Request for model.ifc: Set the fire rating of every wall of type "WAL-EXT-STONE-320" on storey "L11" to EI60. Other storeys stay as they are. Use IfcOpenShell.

First a look at what the model holds.

```python
import ifcopenshell
import ifcopenshell.util.element

model = ifcopenshell.open("model.ifc")
print(model.schema)
storey = next(s for s in model.by_type("IfcBuildingStorey") if s.Name == "L11")
walls = [e for e in ifcopenshell.util.element.get_decomposition(storey) if e.is_a("IfcWall")]
seen = {}
for e in walls:
    element_type = ifcopenshell.util.element.get_type(e)
    key = (element_type.Name if element_type != e and element_type else None, ifcopenshell.util.element.get_pset(e, "Pset_WallCommon", "FireRating"))
    seen[key] = seen.get(key, 0) + 1
for (name, value), count in sorted(seen.items(), key=str):
    print(count, "x", name, "|", value)
```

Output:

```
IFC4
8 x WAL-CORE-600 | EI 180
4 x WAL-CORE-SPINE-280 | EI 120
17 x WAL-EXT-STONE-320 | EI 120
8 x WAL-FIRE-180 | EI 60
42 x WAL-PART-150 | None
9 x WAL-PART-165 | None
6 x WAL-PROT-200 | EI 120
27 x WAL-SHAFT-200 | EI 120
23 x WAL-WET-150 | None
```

```python
import ifcopenshell
import ifcopenshell.api.pset
import ifcopenshell.util.element

model = ifcopenshell.open("model.ifc")

storey = next(s for s in model.by_type("IfcBuildingStorey") if s.Name == "L11")
walls = [e for e in ifcopenshell.util.element.get_decomposition(storey) if e.is_a("IfcWall")]

count = 0
for e in walls:
    element_type = ifcopenshell.util.element.get_type(e)
    if element_type in (None, e) or element_type.Name != "WAL-EXT-STONE-320":
        continue
    # add_pset returns the element's existing set when there is one.
    pset = ifcopenshell.api.pset.add_pset(model, product=e, name="Pset_WallCommon")
    ifcopenshell.api.pset.edit_pset(model, pset=pset, properties={"FireRating": "EI60"})
    count += 1

print(count, "walls updated")

model.write("model_v2.ifc")
```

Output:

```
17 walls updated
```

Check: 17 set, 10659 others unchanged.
